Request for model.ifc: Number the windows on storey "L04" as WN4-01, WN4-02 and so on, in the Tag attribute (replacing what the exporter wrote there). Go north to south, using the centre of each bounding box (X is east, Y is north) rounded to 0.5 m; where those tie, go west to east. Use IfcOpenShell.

First a look at what the model holds.

```python
import ifcopenshell
import ifcopenshell.util.element
import ifcopenshell.util.placement

model = ifcopenshell.open("model.ifc")
print(model.schema)
storey = next(s for s in model.by_type("IfcBuildingStorey") if s.Name == "L04")
windows = [e for e in ifcopenshell.util.element.get_decomposition(storey) if e.is_a("IfcWindow")]
for e in sorted(windows, key=lambda e: e.id()):
    origin = ifcopenshell.util.placement.get_local_placement(e.ObjectPlacement)[:3, 3]
    print(e.id(), e.Tag, e.Name, origin.round(2) + 0.0, sep=" | ")
```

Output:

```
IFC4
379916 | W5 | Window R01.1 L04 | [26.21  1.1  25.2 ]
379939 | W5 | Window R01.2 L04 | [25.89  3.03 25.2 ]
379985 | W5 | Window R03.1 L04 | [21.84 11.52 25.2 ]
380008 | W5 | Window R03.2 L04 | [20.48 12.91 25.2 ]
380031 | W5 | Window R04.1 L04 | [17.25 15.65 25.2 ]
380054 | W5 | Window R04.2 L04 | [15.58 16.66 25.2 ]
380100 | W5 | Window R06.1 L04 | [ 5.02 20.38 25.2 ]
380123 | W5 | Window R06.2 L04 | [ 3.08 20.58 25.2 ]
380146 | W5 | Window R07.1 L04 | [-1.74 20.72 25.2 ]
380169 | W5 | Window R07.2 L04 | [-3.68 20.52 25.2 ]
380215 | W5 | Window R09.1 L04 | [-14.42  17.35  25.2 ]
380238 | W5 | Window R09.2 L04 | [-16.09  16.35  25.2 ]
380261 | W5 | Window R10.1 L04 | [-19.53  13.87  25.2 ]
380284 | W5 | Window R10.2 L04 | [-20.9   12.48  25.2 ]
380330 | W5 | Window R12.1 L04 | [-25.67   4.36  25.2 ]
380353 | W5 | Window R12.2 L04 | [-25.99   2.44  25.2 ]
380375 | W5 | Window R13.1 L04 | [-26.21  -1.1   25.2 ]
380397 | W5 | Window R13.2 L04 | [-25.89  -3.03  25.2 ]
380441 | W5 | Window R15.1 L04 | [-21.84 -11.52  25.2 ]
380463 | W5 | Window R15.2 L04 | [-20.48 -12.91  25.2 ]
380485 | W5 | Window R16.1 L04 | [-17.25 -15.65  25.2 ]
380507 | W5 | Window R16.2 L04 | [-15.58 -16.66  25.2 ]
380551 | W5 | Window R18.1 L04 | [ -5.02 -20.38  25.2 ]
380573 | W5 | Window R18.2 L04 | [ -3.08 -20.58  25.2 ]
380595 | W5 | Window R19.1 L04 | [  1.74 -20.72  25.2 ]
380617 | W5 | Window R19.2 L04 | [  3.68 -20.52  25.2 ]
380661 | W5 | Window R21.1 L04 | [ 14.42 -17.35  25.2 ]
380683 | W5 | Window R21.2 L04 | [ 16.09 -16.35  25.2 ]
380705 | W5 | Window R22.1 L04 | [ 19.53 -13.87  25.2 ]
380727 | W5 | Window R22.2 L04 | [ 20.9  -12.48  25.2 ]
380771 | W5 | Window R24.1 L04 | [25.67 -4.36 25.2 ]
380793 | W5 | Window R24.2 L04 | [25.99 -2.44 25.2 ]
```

```python
import ifcopenshell
import ifcopenshell.geom
import ifcopenshell.util.element
import ifcopenshell.util.shape

model = ifcopenshell.open("model.ifc")
settings = ifcopenshell.geom.settings()
settings.set("use-world-coords", True)


def centre(element):
    shape = ifcopenshell.geom.create_shape(settings, element)
    return ifcopenshell.util.shape.get_bbox_centroid(shape.geometry)


storey = next(s for s in model.by_type("IfcBuildingStorey") if s.Name == "L04")
windows = [e for e in ifcopenshell.util.element.get_decomposition(storey) if e.is_a("IfcWindow")]

# Insertion points can sit at a corner or the storey origin, so sort by the geometry (in metres).
centres = {e: centre(e) for e in windows}
windows.sort(key=lambda e: (-round(centres[e][1] / 0.5), centres[e][0]))

for i, e in enumerate(windows, start=1):
    number = f"WN4-{i:02d}"
    e.Tag = number
    print(e.id(), number)

model.write("model_v2.ifc")
```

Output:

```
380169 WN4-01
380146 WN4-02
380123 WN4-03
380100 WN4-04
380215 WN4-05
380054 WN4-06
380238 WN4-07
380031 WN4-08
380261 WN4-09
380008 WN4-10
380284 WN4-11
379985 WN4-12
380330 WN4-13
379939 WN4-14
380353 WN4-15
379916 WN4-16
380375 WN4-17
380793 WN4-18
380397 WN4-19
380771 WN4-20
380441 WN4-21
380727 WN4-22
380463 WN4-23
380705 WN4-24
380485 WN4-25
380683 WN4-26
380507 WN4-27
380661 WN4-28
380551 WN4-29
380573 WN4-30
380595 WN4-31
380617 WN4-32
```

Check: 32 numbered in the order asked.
